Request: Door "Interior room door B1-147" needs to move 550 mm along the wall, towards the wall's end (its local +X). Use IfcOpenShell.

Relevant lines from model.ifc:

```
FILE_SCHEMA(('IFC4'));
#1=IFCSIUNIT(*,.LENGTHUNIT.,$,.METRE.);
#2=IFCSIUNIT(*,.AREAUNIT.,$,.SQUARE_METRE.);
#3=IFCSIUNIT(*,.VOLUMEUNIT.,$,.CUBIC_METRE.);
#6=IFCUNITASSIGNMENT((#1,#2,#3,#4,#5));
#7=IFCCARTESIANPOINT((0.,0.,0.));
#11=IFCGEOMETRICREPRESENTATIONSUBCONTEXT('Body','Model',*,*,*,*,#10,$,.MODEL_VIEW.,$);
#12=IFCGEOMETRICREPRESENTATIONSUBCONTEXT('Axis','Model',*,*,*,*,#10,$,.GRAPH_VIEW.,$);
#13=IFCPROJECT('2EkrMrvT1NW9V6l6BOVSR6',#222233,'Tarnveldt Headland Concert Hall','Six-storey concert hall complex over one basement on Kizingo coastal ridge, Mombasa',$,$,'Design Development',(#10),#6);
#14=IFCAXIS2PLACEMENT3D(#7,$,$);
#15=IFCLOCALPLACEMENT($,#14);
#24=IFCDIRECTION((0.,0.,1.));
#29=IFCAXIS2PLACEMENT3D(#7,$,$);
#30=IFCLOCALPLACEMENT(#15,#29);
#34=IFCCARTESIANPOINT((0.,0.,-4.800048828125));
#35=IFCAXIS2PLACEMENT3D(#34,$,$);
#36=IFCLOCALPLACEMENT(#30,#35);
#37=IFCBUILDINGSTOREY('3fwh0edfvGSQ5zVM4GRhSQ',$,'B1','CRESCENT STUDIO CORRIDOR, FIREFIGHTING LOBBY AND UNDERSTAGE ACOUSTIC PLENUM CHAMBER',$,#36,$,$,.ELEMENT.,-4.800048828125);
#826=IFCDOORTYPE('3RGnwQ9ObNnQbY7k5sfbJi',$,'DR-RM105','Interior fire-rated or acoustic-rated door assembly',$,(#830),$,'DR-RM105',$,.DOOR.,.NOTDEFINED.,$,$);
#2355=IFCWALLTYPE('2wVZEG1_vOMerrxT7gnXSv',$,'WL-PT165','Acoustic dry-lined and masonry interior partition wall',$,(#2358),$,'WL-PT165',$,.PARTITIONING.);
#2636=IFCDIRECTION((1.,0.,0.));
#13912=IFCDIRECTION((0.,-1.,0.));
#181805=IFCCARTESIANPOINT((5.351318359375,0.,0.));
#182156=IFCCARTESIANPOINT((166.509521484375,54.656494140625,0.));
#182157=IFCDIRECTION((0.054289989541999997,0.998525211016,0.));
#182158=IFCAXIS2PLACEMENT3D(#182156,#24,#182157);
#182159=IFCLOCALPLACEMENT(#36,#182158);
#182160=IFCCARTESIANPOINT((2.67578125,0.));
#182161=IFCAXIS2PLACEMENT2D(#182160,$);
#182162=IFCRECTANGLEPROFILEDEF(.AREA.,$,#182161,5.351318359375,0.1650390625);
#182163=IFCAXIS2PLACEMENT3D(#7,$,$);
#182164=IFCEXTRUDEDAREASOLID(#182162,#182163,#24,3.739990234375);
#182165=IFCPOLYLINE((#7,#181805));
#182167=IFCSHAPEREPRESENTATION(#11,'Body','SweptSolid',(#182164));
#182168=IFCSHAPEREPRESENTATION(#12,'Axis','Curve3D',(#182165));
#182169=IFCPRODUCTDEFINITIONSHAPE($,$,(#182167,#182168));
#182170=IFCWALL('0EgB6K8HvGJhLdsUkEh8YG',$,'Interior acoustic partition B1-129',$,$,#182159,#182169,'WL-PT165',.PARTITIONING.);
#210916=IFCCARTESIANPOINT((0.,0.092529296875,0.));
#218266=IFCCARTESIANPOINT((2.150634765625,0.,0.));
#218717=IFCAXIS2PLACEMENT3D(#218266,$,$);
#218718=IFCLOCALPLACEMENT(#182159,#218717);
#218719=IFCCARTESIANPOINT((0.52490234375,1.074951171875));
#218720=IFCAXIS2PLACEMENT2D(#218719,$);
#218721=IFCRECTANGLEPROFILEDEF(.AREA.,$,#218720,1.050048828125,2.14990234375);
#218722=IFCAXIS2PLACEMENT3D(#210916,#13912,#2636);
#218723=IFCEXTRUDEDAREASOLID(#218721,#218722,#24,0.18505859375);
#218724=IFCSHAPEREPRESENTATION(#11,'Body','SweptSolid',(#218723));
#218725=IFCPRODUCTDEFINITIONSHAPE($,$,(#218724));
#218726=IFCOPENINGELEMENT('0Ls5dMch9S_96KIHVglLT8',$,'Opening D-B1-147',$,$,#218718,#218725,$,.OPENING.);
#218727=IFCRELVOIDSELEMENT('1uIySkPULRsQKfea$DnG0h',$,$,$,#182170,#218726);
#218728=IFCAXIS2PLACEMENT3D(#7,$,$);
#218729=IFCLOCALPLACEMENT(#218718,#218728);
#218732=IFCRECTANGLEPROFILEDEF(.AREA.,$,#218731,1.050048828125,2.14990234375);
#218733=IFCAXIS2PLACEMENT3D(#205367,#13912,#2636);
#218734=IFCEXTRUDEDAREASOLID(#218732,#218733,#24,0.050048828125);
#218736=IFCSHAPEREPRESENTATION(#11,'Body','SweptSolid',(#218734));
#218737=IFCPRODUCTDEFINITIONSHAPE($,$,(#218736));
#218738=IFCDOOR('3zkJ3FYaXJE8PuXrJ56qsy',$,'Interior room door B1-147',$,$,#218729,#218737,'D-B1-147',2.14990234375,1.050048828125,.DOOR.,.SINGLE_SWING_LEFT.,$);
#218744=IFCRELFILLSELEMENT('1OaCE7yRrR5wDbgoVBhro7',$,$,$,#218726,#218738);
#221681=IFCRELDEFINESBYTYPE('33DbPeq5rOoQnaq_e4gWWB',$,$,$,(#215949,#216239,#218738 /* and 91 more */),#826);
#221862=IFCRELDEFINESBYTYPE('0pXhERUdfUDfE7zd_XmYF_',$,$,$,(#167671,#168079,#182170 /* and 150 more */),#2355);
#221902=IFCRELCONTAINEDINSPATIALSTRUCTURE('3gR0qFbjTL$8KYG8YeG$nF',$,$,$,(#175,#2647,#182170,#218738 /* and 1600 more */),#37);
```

```python
import ifcopenshell
import ifcopenshell.api.geometry
import ifcopenshell.util.placement
import ifcopenshell.util.unit

model = ifcopenshell.open("model.ifc")
unit_scale = ifcopenshell.util.unit.calculate_unit_scale(model)

door = model.by_guid("3zkJ3FYaXJE8PuXrJ56qsy")
opening = door.FillsVoids[0].RelatingOpeningElement
wall = opening.VoidsElements[0].RelatingBuildingElement

wall_matrix = ifcopenshell.util.placement.get_local_placement(wall.ObjectPlacement)
shift = wall_matrix[:3, 0] * 0.55 / unit_scale
before = ifcopenshell.util.placement.get_local_placement(door.ObjectPlacement)[:3, 3].copy()

# The door is placed relative to its opening, so it follows when the opening moves.
matrix = ifcopenshell.util.placement.get_local_placement(opening.ObjectPlacement)
matrix[:3, 3] += shift
ifcopenshell.api.geometry.edit_object_placement(
    model, product=opening, matrix=matrix, is_si=False, should_transform_children=True
)

after = ifcopenshell.util.placement.get_local_placement(door.ObjectPlacement)[:3, 3]
print("door moved by", (after - before).round(3) + 0.0)

model.write("model_updated.ifc")
```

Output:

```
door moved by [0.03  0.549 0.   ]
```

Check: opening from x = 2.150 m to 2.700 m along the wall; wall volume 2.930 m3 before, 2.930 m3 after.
